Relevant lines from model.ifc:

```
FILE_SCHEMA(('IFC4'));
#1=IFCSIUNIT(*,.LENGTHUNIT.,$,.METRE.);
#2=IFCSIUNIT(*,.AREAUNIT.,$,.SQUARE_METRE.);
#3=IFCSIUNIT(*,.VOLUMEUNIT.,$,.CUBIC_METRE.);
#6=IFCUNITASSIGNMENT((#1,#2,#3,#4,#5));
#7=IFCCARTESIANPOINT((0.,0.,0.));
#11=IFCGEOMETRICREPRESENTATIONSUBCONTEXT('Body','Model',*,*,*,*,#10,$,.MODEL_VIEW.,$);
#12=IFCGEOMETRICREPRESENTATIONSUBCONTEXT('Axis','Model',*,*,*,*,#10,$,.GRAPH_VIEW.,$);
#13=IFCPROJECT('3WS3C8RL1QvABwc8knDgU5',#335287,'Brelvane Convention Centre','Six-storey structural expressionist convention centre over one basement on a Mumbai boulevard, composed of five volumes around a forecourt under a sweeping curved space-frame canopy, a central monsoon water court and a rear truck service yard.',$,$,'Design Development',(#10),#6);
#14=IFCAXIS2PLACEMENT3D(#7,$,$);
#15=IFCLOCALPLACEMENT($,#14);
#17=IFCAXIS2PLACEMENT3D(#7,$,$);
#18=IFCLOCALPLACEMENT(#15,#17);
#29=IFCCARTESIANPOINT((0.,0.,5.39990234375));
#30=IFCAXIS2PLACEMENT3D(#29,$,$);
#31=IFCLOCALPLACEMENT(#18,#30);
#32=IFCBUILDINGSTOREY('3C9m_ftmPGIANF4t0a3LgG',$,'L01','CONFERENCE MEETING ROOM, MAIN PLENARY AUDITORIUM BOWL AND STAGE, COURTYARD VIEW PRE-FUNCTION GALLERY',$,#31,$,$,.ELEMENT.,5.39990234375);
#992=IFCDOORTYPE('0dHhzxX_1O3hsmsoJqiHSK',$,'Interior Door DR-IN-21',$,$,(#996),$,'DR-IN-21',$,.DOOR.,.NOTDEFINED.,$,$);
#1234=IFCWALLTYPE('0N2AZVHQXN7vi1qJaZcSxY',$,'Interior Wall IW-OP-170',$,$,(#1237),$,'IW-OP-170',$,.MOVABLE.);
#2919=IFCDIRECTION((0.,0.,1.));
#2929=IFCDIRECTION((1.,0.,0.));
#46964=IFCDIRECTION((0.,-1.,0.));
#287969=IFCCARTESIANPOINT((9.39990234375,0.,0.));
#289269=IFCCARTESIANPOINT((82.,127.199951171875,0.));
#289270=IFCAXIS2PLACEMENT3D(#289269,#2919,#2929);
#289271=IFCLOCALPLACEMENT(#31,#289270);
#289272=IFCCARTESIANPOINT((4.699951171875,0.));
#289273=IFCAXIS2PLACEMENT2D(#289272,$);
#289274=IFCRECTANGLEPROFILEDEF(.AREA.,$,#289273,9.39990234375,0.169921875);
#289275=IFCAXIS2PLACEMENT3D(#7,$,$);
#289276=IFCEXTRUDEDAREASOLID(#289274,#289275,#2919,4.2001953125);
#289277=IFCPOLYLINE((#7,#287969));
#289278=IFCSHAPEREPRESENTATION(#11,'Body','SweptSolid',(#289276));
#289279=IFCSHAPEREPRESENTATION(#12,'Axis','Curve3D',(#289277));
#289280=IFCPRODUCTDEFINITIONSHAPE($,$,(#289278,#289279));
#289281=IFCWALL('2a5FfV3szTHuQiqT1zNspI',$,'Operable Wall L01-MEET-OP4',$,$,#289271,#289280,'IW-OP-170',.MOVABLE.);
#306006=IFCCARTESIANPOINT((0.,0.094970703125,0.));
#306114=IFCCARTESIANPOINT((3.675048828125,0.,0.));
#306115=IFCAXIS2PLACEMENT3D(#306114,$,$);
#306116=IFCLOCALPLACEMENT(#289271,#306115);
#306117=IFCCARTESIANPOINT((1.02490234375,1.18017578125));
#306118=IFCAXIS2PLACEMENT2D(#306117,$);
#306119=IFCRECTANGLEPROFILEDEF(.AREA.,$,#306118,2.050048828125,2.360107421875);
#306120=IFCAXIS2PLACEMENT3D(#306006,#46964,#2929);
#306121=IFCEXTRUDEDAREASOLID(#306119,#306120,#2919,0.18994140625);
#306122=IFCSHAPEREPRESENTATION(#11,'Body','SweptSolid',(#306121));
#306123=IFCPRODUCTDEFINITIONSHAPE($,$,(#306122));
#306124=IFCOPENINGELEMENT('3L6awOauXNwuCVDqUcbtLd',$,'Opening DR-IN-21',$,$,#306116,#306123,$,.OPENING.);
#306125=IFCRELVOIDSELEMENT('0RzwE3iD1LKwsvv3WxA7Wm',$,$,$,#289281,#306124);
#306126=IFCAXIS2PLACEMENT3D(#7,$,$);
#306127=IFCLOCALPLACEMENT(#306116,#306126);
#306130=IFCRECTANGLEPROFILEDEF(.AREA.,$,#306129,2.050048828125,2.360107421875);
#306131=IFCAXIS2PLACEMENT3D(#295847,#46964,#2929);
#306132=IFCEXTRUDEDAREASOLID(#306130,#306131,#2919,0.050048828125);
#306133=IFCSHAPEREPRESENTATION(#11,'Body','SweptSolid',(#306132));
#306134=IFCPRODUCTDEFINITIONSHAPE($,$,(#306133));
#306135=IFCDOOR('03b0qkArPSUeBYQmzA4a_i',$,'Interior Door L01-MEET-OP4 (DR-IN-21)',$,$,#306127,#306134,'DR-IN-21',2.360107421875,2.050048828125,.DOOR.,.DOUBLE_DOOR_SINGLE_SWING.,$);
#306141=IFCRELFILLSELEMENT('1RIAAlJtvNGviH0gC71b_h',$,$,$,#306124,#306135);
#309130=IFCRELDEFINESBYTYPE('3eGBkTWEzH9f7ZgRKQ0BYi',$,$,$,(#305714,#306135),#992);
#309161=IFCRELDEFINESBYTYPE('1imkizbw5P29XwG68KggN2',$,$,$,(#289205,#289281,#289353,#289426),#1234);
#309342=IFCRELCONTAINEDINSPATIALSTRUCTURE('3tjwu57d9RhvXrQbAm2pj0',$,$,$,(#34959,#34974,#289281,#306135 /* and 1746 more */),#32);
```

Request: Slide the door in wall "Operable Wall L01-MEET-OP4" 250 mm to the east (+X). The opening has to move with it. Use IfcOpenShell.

```python
import ifcopenshell
import ifcopenshell.api.geometry
import ifcopenshell.util.placement
import ifcopenshell.util.unit

model = ifcopenshell.open("model.ifc")
unit_scale = ifcopenshell.util.unit.calculate_unit_scale(model)

door = model.by_guid("03b0qkArPSUeBYQmzA4a_i")
opening = door.FillsVoids[0].RelatingOpeningElement
wall = opening.VoidsElements[0].RelatingBuildingElement

wall_matrix = ifcopenshell.util.placement.get_local_placement(wall.ObjectPlacement)
shift = wall_matrix[:3, 0] * 0.25 / unit_scale
before = ifcopenshell.util.placement.get_local_placement(door.ObjectPlacement)[:3, 3].copy()

# The door is placed relative to its opening, so it follows when the opening moves.
matrix = ifcopenshell.util.placement.get_local_placement(opening.ObjectPlacement)
matrix[:3, 3] += shift
ifcopenshell.api.geometry.edit_object_placement(
    model, product=opening, matrix=matrix, is_si=False, should_transform_children=True
)

after = ifcopenshell.util.placement.get_local_placement(door.ObjectPlacement)[:3, 3]
print("door moved by", (after - before).round(3) + 0.0)

model.write("model_edited.ifc")
```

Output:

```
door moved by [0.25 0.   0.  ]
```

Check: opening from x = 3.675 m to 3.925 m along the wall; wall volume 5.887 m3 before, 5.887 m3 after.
